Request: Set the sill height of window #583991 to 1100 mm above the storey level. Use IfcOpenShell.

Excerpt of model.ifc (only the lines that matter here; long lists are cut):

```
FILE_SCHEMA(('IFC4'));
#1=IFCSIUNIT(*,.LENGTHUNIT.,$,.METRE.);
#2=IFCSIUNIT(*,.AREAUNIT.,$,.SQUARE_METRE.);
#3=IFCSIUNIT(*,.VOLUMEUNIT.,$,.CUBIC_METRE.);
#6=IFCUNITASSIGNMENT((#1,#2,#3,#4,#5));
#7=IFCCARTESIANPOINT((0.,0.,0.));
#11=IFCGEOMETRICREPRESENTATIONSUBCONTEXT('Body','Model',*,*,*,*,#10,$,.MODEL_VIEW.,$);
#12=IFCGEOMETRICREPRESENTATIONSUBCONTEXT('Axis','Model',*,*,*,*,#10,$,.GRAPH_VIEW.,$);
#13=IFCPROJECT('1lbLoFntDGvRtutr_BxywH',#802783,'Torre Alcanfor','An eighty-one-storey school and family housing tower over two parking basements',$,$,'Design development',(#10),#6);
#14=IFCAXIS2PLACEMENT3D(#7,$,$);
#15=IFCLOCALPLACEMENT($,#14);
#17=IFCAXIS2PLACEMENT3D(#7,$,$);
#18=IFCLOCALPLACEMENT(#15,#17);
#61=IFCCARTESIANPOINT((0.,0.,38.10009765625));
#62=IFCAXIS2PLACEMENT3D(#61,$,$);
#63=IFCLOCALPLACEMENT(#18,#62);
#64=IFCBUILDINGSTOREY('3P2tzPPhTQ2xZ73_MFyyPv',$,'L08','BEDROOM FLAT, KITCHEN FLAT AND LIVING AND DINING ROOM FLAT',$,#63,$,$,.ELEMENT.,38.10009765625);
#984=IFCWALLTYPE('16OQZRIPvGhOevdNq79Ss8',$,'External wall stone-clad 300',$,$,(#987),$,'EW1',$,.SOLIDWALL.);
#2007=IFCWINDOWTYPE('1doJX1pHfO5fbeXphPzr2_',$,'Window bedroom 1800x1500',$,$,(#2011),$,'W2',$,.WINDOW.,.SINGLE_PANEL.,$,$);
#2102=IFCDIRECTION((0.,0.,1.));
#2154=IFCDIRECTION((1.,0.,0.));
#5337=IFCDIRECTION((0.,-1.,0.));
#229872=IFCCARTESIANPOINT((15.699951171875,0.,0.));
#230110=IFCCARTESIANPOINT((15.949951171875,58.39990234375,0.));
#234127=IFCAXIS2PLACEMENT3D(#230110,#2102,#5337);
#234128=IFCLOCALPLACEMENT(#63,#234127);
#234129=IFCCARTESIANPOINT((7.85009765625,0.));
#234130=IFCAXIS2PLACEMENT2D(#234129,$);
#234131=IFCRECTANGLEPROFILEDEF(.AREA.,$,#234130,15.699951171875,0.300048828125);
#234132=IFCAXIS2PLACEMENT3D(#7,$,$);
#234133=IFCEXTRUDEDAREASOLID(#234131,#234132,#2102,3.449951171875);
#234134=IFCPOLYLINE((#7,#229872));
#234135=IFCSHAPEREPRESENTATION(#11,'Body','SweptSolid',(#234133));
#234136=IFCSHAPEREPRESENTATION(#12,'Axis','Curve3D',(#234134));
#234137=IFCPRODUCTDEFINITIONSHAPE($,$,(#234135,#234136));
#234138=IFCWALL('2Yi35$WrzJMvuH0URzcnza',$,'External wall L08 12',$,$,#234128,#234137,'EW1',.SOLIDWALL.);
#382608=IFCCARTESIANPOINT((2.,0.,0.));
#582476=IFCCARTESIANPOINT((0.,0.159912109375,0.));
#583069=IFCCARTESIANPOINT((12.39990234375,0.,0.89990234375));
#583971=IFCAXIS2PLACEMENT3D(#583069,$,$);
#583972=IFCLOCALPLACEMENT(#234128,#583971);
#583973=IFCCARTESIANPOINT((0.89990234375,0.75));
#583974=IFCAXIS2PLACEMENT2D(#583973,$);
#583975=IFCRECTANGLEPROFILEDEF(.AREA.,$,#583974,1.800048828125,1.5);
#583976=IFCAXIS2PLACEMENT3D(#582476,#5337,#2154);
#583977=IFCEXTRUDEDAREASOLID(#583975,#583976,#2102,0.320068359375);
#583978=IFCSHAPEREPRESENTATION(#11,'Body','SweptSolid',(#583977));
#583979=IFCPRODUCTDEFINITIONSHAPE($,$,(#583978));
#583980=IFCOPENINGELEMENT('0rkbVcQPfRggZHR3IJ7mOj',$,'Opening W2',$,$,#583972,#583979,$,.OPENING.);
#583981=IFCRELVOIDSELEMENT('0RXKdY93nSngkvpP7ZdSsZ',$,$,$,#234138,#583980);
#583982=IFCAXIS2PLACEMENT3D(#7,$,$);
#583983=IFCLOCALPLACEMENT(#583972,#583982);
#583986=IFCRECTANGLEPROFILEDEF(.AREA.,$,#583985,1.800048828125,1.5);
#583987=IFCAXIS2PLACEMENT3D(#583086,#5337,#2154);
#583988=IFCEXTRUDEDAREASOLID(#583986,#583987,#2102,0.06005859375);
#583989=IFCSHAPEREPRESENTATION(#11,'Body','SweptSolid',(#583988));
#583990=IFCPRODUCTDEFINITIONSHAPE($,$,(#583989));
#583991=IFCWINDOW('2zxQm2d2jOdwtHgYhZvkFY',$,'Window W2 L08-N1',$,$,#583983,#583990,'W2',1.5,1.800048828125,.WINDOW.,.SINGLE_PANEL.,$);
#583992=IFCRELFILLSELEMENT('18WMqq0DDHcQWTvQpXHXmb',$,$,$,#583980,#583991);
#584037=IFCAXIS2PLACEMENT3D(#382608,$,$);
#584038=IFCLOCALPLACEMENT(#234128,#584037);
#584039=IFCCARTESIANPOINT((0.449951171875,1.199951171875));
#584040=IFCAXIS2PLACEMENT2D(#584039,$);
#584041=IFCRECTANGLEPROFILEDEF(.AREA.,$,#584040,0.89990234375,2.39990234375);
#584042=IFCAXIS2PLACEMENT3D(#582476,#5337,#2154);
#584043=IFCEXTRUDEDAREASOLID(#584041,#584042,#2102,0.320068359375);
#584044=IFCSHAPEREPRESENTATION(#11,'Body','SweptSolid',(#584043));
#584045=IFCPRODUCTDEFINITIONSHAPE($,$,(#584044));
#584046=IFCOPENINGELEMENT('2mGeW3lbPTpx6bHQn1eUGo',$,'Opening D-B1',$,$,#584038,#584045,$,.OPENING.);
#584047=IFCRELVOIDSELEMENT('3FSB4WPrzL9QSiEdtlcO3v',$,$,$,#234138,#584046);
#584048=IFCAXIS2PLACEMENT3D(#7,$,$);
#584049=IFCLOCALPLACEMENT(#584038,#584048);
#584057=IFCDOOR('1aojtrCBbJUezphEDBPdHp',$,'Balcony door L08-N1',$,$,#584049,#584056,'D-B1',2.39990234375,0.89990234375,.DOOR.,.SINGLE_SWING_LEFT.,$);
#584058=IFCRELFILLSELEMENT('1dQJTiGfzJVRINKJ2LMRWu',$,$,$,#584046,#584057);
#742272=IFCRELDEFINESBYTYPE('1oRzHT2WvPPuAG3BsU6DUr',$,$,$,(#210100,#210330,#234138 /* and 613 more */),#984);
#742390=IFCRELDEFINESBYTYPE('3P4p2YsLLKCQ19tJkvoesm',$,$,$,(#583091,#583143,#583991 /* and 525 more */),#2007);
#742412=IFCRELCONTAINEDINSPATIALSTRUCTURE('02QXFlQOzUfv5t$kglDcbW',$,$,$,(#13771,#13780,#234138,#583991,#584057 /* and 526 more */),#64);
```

```python
import numpy as np
import ifcopenshell
import ifcopenshell.api.geometry
import ifcopenshell.geom
import ifcopenshell.util.element
import ifcopenshell.util.placement
import ifcopenshell.util.shape
import ifcopenshell.util.unit

model = ifcopenshell.open("model.ifc")
unit_scale = ifcopenshell.util.unit.calculate_unit_scale(model)

window = model.by_guid("2zxQm2d2jOdwtHgYhZvkFY")
opening = window.FillsVoids[0].RelatingOpeningElement
storey = ifcopenshell.util.element.get_container(window, ifc_class="IfcBuildingStorey")
level = ifcopenshell.util.placement.get_local_placement(storey.ObjectPlacement)[2, 3]

# The opening's origin need not be at the sill, so measure its lowest point.
shape = ifcopenshell.geom.create_shape(ifcopenshell.geom.settings(), opening)
bottom = ifcopenshell.util.shape.get_shape_bottom_elevation(shape, shape.geometry) / unit_scale
dz = level + 1.1 / unit_scale - bottom

shift = np.array([0.0, 0.0, dz])
# The window is placed relative to its opening, so it follows when the opening moves.
matrix = ifcopenshell.util.placement.get_local_placement(opening.ObjectPlacement)
matrix[:3, 3] += shift
ifcopenshell.api.geometry.edit_object_placement(
    model, product=opening, matrix=matrix, is_si=False, should_transform_children=True
)

print(f"moved by {dz * unit_scale:+.3f} m")

model.write("model_edited.ifc")
```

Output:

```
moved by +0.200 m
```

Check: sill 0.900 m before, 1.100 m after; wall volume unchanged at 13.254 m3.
